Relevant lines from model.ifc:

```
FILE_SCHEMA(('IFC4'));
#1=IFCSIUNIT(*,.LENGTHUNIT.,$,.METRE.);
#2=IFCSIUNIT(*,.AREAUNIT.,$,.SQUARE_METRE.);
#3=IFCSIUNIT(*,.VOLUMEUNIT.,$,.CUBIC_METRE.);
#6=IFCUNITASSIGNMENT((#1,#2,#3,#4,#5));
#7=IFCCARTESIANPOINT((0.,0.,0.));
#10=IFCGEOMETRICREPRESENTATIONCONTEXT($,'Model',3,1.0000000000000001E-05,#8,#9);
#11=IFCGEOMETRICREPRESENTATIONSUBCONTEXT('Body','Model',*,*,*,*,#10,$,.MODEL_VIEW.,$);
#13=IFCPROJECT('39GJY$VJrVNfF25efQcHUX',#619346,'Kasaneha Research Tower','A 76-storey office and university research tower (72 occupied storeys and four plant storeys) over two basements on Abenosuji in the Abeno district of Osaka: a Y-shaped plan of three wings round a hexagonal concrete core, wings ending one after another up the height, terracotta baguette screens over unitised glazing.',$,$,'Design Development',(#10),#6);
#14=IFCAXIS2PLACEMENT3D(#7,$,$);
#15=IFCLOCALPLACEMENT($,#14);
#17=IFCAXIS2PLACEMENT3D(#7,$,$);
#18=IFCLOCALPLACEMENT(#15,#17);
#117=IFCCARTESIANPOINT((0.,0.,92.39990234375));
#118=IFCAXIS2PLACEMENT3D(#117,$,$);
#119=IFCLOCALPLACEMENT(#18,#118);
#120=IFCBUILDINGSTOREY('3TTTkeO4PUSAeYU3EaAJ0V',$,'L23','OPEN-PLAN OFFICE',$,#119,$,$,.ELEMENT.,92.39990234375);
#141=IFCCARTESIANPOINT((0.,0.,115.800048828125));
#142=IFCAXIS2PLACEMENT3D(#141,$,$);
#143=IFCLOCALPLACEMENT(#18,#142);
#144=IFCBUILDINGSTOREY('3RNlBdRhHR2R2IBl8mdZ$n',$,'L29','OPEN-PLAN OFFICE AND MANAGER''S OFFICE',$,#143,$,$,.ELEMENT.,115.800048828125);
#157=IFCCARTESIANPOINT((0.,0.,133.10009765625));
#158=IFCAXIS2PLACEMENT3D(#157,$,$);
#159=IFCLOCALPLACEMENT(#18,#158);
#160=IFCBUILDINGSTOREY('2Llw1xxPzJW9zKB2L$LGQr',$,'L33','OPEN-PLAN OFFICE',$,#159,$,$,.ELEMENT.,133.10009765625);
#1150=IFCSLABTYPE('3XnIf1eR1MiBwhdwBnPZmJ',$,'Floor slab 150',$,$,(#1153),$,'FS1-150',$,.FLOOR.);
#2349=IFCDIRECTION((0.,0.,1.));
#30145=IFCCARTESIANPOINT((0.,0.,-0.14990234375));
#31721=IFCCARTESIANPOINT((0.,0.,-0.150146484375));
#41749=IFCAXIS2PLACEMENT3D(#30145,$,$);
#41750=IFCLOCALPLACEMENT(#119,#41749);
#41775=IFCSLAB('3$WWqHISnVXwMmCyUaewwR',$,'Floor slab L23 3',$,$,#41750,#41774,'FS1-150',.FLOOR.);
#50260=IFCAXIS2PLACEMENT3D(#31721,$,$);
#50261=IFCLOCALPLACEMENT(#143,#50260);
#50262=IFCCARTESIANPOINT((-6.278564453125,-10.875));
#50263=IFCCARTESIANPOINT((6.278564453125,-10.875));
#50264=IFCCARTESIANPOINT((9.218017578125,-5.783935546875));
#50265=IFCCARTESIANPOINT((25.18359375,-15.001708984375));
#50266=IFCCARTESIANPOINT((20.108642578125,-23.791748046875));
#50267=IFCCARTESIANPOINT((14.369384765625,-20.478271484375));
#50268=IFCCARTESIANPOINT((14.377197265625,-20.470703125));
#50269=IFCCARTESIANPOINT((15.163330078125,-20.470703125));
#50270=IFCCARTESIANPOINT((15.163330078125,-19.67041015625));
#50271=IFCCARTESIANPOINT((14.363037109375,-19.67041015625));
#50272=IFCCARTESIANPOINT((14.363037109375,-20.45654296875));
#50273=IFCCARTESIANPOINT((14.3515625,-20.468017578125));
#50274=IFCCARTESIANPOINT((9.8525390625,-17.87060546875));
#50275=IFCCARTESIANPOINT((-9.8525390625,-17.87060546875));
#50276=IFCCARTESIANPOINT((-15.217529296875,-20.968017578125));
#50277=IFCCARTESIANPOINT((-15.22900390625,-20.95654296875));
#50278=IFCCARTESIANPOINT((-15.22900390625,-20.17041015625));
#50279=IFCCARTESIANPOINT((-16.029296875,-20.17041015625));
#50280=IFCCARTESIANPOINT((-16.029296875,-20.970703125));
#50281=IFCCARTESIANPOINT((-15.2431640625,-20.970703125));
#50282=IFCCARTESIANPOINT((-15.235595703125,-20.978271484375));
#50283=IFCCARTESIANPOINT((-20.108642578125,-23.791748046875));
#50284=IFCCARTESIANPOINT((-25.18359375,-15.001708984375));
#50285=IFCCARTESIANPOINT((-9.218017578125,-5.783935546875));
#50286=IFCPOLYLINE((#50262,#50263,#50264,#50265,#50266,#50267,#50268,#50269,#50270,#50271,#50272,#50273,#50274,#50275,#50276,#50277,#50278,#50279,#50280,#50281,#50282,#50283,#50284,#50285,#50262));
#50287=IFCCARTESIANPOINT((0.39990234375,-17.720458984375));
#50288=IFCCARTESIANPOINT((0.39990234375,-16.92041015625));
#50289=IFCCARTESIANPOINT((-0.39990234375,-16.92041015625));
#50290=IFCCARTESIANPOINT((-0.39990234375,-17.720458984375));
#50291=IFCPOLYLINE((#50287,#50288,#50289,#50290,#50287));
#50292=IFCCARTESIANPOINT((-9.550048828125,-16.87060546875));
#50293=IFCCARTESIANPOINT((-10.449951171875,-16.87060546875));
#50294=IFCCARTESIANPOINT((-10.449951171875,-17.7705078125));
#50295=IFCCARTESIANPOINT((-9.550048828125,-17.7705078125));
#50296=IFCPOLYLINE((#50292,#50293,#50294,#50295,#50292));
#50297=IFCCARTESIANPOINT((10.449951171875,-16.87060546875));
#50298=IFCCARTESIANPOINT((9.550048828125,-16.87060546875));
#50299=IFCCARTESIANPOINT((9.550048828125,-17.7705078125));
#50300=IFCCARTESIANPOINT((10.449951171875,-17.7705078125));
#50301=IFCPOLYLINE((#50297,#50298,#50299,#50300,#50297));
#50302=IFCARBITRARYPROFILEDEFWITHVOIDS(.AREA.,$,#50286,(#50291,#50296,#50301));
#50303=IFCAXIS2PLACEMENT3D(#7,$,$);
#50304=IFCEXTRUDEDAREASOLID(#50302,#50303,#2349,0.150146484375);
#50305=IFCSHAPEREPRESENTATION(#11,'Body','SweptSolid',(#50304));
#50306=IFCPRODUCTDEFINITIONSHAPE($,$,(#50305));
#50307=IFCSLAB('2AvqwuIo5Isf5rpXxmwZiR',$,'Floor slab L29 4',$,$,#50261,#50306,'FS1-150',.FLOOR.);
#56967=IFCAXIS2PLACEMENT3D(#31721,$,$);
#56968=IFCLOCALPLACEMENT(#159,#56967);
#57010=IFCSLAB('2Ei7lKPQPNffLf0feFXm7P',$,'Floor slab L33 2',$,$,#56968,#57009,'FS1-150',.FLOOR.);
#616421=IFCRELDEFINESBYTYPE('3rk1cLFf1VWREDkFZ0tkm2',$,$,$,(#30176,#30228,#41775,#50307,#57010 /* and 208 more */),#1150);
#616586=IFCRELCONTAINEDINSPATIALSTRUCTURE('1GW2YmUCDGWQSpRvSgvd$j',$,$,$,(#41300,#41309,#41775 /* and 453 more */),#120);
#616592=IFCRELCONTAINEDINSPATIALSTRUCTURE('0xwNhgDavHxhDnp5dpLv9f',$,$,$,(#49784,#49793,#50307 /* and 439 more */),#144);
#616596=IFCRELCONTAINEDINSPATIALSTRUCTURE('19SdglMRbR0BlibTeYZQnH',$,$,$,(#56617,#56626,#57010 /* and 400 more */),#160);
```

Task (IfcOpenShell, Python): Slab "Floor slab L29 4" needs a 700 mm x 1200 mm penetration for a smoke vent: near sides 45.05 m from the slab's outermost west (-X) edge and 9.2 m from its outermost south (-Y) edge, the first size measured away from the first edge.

```python
import numpy as np
import ifcopenshell
import ifcopenshell.api.feature
import ifcopenshell.api.geometry
import ifcopenshell.api.root
import ifcopenshell.geom
import ifcopenshell.util.placement
import ifcopenshell.util.representation
import ifcopenshell.util.shape
import ifcopenshell.util.unit

model = ifcopenshell.open("model.ifc")
unit_scale = ifcopenshell.util.unit.calculate_unit_scale(model)
settings = ifcopenshell.geom.settings()


def volume(element):
    """Net volume in cubic metres, openings subtracted."""
    shape = ifcopenshell.geom.create_shape(settings, element)
    return ifcopenshell.util.shape.get_volume(shape.geometry)


slab = model.by_id(50307)
before = volume(slab)

# Extent in the slab's own axes, in metres. The edges named are its -X and -Y sides.
slab_shape = ifcopenshell.geom.create_shape(settings, slab)
vertices = ifcopenshell.util.shape.get_vertices(slab_shape.geometry)
x_min, y_min, bottom = vertices.min(axis=0)
top = vertices[:, 2].max()

opening = ifcopenshell.api.root.create_entity(model, ifc_class="IfcOpeningElement", name="Smoke vent opening", predefined_type="OPENING")
context = ifcopenshell.util.representation.get_context(model, "Model", "Body", "MODEL_VIEW")
width, depth = 0.7, 1.2
outline = [(0.0, 0.0), (width, 0.0), (width, depth), (0.0, depth), (0.0, 0.0)]
# Overshoot both faces by 50 mm so the cut is clean.
shape = ifcopenshell.api.geometry.add_slab_representation(
    model, context=context, depth=top - bottom + 0.1, polyline=outline
)
ifcopenshell.api.geometry.assign_representation(model, product=opening, representation=shape)

matrix = ifcopenshell.util.placement.get_local_placement(slab.ObjectPlacement)
matrix[:, 3] = matrix @ np.append(np.array([x_min + 45.05, y_min + 9.2, bottom - 0.05]) / unit_scale, 1.0)
ifcopenshell.api.geometry.edit_object_placement(model, product=opening, matrix=matrix, is_si=False)
ifcopenshell.api.feature.add_feature(model, feature=opening, element=slab)

after = volume(slab)

print(f"slab volume {before:.3f} -> {after:.3f} m3")

model.write("model_v2.ifc")
```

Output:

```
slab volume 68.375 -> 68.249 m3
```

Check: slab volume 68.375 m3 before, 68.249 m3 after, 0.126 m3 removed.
